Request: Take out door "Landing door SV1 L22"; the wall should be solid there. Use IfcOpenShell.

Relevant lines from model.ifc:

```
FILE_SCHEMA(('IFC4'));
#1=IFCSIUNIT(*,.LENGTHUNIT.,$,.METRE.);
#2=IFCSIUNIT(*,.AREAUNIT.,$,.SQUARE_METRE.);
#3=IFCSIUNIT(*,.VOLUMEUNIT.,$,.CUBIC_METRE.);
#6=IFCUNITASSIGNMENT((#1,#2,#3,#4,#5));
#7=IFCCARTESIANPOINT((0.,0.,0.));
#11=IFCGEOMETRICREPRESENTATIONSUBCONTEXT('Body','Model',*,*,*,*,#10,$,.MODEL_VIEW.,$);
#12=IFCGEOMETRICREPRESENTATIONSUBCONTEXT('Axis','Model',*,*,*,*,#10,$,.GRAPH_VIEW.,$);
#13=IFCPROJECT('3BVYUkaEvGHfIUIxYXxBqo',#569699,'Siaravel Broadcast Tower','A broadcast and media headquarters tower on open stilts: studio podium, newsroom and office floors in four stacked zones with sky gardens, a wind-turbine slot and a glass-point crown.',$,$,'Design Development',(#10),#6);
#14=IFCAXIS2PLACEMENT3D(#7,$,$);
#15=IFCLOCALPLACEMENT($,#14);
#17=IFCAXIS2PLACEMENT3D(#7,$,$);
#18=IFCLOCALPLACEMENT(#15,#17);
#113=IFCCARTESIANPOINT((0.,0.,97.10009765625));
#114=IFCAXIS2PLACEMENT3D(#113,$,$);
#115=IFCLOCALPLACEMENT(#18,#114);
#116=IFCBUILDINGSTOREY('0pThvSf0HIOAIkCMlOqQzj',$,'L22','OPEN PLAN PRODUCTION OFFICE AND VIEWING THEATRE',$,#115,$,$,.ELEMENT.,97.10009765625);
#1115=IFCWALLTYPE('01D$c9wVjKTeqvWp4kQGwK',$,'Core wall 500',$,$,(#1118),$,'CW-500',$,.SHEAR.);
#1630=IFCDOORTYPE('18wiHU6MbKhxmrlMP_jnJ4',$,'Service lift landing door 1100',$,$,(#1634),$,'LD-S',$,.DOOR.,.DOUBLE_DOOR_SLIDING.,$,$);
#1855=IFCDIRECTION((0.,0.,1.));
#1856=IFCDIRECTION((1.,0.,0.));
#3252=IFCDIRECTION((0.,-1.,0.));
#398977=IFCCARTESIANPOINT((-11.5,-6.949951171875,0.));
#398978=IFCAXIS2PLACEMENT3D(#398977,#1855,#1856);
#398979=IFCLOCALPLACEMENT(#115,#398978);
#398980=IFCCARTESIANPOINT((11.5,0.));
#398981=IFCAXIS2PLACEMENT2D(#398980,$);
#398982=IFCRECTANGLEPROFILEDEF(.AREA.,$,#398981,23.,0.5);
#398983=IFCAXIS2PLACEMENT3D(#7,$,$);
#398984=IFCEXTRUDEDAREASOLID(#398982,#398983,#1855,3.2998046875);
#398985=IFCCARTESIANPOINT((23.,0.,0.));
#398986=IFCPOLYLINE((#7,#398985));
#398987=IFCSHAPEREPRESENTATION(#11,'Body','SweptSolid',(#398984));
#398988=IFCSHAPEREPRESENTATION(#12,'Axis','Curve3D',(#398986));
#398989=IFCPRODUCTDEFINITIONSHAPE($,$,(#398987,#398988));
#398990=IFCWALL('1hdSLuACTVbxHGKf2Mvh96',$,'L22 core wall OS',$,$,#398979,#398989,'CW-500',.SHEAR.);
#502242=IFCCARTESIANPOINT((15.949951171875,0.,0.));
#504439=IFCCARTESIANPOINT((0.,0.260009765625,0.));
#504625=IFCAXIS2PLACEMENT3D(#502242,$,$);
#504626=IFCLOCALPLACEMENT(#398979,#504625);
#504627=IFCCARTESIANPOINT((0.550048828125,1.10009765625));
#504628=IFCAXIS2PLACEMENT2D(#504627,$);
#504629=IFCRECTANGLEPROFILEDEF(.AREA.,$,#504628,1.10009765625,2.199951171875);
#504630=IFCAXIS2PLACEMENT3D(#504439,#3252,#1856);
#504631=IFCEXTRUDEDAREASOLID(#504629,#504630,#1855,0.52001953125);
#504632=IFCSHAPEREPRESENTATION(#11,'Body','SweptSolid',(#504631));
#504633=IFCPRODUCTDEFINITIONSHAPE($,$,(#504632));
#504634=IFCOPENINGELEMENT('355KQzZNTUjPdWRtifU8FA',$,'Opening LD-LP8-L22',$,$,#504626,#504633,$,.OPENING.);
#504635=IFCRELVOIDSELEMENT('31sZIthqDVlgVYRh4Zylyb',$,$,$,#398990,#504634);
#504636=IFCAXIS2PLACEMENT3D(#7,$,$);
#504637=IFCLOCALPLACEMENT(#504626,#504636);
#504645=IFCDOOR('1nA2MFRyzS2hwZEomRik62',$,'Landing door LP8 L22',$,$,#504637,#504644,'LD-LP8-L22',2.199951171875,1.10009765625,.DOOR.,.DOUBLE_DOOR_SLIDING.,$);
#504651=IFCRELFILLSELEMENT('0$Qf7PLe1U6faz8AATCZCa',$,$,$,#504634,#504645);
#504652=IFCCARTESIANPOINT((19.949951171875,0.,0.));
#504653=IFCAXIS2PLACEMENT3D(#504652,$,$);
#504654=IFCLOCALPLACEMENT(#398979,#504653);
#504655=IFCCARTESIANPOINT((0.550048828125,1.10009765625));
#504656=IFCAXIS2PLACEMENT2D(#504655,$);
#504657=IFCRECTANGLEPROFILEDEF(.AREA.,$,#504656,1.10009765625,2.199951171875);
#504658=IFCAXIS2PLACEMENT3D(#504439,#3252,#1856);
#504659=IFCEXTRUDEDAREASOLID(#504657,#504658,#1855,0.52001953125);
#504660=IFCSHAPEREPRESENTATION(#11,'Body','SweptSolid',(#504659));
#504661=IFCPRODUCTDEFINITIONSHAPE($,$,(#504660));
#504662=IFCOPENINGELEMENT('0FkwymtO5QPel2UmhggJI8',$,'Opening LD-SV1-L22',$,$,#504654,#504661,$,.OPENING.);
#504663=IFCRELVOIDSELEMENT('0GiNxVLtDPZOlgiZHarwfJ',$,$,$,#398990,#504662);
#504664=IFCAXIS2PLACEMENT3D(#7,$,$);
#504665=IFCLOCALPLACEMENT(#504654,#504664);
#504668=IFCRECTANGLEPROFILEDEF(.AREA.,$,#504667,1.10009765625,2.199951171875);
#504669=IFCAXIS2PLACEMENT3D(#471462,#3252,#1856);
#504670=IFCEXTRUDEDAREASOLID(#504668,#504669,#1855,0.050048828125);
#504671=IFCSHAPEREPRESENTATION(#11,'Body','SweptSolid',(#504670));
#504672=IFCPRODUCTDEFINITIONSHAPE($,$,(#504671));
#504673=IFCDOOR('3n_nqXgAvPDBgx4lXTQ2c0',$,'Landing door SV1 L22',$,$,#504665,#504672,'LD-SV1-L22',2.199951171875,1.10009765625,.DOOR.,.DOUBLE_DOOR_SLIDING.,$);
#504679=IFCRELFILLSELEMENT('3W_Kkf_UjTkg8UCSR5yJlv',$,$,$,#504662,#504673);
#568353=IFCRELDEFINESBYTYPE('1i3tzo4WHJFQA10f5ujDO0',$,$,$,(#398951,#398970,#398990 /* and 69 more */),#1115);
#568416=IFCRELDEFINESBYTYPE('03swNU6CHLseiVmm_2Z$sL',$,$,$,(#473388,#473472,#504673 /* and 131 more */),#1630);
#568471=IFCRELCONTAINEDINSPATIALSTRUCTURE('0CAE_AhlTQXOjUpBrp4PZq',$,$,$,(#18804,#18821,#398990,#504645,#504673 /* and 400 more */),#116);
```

```python
import ifcopenshell
import ifcopenshell.api.feature
import ifcopenshell.api.root
import ifcopenshell.geom
import ifcopenshell.util.shape

model = ifcopenshell.open("model.ifc")
settings = ifcopenshell.geom.settings()


def volume(element):
    """Net volume in cubic metres, openings subtracted."""
    shape = ifcopenshell.geom.create_shape(settings, element)
    return ifcopenshell.util.shape.get_volume(shape.geometry)


door = model.by_id(504673)
opening = door.FillsVoids[0].RelatingOpeningElement
wall = opening.VoidsElements[0].RelatingBuildingElement
before = volume(wall)

ifcopenshell.api.root.remove_product(model, product=door)
ifcopenshell.api.feature.remove_feature(model, feature=opening)

after = volume(wall)

print(f"wall volume {before:.3f} -> {after:.3f} m3")

model.write("model_rev.ifc")
```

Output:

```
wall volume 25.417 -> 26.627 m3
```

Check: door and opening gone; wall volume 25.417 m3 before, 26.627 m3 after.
